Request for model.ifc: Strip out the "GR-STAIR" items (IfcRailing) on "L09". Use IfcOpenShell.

First a look at what the model holds.

```python
import ifcopenshell
import ifcopenshell.util.element

model = ifcopenshell.open("model.ifc")
print(model.schema)
storey = next(s for s in model.by_type("IfcBuildingStorey") if s.Name == "L09")
railings = [e for e in ifcopenshell.util.element.get_decomposition(storey) if e.is_a("IfcRailing")]
seen = {}
for e in railings:
    element_type = ifcopenshell.util.element.get_type(e)
    name = element_type.Name if element_type not in (None, e) else None
    seen[name] = seen.get(name, 0) + 1
for name, count in sorted(seen.items(), key=str):
    print(count, "x", name)
```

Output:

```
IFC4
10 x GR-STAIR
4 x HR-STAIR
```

```python
import ifcopenshell
import ifcopenshell.api.root
import ifcopenshell.util.element

model = ifcopenshell.open("model.ifc")

storey = next(s for s in model.by_type("IfcBuildingStorey") if s.Name == "L09")
railings = [e for e in ifcopenshell.util.element.get_decomposition(storey) if e.is_a("IfcRailing")]
targets = [e for e in railings if (t := ifcopenshell.util.element.get_type(e)) not in (None, e) and t.Name == "GR-STAIR"]

for e in targets:
    ifcopenshell.api.root.remove_product(model, product=e)
print(len(targets), "removed")

model.write("model_rev.ifc")
```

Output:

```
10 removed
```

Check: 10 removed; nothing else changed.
